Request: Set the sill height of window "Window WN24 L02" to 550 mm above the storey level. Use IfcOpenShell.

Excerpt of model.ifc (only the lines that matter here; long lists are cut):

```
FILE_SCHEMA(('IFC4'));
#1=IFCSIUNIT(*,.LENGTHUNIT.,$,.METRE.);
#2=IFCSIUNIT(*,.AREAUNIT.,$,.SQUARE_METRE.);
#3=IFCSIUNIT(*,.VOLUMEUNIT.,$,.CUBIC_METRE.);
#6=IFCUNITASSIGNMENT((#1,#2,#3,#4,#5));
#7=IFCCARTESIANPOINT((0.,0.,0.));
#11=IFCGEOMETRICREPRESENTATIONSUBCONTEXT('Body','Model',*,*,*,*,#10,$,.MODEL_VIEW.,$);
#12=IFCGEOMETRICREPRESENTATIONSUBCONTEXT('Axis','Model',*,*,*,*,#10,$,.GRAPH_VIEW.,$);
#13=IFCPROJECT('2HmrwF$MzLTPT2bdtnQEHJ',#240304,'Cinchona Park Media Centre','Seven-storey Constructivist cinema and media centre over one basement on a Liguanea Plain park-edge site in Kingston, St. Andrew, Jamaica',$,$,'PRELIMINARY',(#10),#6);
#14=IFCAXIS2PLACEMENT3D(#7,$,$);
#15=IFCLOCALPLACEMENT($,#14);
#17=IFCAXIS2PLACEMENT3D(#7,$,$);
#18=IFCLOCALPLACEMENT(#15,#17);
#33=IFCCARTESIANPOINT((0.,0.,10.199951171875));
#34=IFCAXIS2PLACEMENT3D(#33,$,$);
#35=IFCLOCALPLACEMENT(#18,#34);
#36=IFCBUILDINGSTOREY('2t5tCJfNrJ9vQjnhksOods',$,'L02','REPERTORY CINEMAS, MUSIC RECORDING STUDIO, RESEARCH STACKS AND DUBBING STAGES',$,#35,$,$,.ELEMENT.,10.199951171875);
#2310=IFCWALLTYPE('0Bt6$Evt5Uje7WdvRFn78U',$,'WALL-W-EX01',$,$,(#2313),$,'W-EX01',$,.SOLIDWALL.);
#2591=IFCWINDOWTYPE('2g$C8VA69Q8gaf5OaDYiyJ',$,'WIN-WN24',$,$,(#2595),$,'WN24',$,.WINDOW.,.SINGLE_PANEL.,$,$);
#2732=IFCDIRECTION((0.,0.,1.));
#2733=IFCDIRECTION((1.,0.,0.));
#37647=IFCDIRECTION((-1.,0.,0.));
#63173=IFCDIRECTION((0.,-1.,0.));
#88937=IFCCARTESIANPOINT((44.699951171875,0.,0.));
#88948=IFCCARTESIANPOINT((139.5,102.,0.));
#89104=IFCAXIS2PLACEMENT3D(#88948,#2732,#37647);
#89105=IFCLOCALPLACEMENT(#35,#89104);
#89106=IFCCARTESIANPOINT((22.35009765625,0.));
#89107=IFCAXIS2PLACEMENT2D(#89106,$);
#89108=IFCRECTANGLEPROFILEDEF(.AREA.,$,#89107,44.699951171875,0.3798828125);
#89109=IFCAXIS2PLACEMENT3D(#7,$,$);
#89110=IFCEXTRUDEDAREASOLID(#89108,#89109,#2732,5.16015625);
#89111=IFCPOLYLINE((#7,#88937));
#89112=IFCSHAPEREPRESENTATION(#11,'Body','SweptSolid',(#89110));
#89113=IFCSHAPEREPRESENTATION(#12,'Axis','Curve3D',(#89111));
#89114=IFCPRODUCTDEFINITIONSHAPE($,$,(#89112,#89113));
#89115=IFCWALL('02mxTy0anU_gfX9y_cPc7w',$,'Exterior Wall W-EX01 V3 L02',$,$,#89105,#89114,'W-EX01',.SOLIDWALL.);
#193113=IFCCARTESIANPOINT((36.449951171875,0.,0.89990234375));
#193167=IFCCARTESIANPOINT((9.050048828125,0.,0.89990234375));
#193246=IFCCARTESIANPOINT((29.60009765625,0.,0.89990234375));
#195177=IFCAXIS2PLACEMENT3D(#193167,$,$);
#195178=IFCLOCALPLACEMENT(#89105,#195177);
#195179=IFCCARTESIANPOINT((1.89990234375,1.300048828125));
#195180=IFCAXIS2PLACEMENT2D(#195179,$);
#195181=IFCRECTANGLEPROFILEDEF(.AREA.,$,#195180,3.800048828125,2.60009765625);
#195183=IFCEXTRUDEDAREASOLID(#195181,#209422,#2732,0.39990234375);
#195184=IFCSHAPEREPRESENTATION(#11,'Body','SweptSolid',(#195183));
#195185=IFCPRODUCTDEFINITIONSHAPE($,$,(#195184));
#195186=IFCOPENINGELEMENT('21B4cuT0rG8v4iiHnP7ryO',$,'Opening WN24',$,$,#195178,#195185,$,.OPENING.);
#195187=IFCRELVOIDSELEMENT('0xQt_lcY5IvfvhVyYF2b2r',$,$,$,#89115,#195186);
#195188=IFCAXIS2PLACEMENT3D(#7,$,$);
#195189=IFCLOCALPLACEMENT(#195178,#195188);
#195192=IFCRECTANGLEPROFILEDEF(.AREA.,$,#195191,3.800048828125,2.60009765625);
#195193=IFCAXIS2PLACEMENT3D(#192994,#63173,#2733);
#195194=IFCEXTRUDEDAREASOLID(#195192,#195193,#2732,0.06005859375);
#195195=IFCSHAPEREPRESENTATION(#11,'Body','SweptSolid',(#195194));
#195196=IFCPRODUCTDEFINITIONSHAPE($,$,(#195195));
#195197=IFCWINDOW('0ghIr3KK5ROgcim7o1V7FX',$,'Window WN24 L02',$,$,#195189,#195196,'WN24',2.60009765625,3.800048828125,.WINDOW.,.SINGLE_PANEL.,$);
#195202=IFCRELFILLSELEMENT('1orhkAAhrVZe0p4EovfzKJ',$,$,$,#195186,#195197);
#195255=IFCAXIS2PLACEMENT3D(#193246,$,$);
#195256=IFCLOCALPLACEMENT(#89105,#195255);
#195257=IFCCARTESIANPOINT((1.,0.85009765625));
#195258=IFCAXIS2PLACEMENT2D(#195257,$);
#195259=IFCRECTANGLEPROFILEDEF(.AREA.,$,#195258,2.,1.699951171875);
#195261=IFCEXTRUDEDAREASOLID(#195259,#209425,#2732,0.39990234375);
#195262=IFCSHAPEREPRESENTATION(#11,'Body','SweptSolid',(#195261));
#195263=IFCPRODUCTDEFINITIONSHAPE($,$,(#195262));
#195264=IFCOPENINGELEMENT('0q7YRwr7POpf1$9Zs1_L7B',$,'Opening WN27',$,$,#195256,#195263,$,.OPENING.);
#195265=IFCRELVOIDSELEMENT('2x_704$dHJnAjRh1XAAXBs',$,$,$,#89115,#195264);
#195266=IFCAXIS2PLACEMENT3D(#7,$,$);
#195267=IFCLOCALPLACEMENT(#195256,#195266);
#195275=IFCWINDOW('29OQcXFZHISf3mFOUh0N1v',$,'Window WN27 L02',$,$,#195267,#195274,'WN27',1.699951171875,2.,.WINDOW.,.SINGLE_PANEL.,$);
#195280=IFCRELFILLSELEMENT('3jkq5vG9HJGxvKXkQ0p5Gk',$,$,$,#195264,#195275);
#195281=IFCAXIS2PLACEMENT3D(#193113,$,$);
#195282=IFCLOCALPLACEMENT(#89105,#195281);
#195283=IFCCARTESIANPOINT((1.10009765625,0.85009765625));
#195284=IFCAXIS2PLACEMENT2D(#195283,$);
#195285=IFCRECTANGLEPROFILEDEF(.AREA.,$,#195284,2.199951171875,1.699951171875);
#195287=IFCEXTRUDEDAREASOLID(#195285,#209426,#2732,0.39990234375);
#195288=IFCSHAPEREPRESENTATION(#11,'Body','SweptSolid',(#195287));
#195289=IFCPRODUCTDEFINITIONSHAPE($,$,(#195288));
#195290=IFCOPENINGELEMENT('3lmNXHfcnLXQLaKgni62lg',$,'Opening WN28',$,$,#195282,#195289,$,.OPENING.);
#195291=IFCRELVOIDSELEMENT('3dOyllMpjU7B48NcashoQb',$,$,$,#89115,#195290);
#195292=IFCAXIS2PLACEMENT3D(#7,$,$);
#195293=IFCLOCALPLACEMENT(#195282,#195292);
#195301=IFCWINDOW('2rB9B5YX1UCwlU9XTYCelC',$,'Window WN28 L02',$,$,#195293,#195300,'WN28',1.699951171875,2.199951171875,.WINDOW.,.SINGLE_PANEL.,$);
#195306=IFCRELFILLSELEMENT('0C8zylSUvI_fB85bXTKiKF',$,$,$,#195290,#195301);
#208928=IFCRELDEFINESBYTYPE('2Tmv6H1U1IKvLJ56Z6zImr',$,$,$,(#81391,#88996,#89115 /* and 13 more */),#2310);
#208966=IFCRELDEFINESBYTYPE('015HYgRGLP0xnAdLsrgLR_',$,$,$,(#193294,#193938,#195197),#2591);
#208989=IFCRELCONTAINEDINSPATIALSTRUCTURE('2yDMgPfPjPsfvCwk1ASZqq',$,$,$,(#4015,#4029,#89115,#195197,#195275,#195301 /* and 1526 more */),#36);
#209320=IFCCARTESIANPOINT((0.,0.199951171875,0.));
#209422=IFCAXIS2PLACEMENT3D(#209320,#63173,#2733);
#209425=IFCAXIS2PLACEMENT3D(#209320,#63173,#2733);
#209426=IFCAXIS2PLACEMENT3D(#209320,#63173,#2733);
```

```python
import numpy as np
import ifcopenshell
import ifcopenshell.api.geometry
import ifcopenshell.geom
import ifcopenshell.util.element
import ifcopenshell.util.placement
import ifcopenshell.util.shape
import ifcopenshell.util.unit

model = ifcopenshell.open("model.ifc")
unit_scale = ifcopenshell.util.unit.calculate_unit_scale(model)

window = model.by_guid("0ghIr3KK5ROgcim7o1V7FX")
opening = window.FillsVoids[0].RelatingOpeningElement
storey = ifcopenshell.util.element.get_container(window, ifc_class="IfcBuildingStorey")
level = ifcopenshell.util.placement.get_local_placement(storey.ObjectPlacement)[2, 3]

# The opening's origin need not be at the sill, so measure its lowest point.
shape = ifcopenshell.geom.create_shape(ifcopenshell.geom.settings(), opening)
bottom = ifcopenshell.util.shape.get_shape_bottom_elevation(shape, shape.geometry) / unit_scale
dz = level + 0.55 / unit_scale - bottom

shift = np.array([0.0, 0.0, dz])
# The window is placed relative to its opening, so it follows when the opening moves.
matrix = ifcopenshell.util.placement.get_local_placement(opening.ObjectPlacement)
matrix[:3, 3] += shift
ifcopenshell.api.geometry.edit_object_placement(
    model, product=opening, matrix=matrix, is_si=False, should_transform_children=True
)

print(f"moved by {dz * unit_scale:+.3f} m")

model.write("model_v2.ifc")
```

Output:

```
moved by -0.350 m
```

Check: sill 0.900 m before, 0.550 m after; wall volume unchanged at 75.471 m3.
